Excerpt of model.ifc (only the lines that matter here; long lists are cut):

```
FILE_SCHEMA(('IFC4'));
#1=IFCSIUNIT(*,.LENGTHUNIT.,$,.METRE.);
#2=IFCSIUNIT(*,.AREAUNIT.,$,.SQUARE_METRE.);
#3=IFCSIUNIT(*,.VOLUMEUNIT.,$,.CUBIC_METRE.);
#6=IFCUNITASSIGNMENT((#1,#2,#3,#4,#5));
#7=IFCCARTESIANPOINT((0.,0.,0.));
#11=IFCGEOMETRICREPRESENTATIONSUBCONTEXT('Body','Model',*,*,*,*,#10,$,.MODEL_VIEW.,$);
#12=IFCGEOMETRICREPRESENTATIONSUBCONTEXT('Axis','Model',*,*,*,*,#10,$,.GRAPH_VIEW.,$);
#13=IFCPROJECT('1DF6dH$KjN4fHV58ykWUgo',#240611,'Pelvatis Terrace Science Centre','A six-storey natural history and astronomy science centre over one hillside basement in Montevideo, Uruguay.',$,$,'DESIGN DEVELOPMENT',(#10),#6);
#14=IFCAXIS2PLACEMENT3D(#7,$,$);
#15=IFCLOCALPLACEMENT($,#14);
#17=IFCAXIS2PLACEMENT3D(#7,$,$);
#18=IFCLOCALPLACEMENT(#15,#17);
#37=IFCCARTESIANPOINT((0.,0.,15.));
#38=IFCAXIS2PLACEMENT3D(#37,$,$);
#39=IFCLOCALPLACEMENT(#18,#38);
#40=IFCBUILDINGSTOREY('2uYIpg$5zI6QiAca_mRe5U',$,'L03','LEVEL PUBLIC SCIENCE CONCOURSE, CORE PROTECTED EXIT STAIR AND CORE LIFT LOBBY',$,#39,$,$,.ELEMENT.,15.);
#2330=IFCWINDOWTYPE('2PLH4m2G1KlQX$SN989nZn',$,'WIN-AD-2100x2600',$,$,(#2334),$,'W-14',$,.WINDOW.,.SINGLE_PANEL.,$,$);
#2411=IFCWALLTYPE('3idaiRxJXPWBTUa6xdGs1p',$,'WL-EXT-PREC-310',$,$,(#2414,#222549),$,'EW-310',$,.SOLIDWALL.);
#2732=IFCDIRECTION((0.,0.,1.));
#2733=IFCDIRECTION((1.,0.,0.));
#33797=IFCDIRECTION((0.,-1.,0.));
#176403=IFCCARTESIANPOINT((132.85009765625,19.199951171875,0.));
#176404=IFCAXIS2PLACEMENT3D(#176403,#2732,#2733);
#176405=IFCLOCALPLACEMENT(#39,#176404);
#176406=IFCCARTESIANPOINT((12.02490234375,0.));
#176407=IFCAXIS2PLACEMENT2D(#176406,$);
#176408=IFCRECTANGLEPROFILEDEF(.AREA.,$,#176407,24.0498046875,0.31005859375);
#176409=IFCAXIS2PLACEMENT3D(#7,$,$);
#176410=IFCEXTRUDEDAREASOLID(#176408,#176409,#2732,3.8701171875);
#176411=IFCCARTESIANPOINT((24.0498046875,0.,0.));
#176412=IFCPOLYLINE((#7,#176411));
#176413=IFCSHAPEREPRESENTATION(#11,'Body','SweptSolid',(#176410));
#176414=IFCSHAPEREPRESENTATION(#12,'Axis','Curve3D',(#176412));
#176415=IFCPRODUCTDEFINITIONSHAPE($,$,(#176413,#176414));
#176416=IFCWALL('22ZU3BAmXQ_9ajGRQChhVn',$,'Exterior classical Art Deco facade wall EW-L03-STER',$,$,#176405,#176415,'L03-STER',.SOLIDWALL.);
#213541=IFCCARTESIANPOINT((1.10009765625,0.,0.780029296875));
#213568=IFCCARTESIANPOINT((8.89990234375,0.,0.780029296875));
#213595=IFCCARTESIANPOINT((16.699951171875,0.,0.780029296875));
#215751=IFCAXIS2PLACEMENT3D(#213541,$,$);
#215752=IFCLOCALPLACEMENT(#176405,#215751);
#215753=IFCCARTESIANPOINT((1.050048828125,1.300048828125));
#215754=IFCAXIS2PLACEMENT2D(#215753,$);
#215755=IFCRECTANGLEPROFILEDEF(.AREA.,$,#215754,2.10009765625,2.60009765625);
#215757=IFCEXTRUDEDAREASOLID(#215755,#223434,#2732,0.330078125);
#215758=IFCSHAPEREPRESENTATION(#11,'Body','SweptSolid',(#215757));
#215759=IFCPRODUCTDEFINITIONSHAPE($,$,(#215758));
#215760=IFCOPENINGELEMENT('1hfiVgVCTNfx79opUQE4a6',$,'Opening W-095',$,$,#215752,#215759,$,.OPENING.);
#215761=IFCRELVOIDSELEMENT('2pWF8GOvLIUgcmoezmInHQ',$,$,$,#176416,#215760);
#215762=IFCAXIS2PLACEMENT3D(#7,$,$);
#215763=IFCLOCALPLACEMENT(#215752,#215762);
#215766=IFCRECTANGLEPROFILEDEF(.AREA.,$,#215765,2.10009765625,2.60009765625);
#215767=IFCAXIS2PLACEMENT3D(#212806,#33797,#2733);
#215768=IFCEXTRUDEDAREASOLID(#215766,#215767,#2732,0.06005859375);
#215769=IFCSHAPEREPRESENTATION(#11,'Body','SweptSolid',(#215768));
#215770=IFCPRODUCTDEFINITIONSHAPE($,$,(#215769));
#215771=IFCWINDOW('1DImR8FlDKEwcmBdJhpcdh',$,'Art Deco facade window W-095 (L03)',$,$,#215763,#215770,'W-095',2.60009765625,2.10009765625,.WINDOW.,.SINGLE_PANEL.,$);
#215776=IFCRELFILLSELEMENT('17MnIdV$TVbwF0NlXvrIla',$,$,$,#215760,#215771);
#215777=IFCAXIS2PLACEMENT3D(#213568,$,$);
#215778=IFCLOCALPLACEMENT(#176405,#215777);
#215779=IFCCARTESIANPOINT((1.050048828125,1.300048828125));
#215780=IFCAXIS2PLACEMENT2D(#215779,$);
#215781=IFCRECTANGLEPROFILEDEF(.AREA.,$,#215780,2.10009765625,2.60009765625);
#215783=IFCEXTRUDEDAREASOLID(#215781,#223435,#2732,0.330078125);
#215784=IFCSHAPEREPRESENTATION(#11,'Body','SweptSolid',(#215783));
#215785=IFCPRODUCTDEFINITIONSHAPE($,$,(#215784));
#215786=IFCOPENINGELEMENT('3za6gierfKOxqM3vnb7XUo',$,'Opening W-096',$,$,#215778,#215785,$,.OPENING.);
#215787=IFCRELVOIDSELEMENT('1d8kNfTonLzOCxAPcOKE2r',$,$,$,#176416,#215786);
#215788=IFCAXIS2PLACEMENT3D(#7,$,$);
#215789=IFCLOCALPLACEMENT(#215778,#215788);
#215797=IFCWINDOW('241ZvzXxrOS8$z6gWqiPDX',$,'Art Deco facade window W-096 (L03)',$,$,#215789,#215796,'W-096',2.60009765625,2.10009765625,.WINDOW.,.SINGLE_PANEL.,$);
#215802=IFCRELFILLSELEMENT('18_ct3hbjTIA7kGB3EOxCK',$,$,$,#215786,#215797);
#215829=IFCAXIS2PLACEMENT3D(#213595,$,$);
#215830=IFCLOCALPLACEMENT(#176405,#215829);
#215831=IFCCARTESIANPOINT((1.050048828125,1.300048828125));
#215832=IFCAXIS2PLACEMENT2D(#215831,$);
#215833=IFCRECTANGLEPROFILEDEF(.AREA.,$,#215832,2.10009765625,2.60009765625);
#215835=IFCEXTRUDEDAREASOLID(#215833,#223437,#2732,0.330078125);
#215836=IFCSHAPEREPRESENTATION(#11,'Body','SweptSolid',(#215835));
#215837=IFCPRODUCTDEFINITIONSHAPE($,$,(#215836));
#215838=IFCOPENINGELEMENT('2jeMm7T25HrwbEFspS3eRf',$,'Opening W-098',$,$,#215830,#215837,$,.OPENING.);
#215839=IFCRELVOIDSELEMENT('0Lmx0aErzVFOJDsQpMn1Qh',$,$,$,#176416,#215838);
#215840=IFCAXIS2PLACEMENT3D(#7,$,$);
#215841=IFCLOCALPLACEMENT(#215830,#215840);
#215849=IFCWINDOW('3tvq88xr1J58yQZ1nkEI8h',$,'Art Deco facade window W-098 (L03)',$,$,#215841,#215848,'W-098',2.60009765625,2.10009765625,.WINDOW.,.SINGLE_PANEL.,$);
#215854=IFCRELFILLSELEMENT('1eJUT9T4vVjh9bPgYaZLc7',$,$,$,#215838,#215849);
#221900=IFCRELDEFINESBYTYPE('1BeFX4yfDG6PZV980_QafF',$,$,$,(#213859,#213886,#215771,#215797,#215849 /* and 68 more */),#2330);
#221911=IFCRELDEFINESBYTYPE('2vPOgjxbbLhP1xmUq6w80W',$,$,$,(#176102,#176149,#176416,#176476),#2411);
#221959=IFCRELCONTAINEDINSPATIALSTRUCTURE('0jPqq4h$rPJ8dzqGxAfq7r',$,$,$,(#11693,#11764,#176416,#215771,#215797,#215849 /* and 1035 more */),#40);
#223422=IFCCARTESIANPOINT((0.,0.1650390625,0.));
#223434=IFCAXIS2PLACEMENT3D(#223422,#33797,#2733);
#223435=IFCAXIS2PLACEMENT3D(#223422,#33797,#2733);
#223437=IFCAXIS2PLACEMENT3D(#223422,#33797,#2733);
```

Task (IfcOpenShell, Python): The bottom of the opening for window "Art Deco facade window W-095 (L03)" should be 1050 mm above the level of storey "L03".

```python
import numpy as np
import ifcopenshell
import ifcopenshell.api.geometry
import ifcopenshell.geom
import ifcopenshell.util.element
import ifcopenshell.util.placement
import ifcopenshell.util.shape
import ifcopenshell.util.unit

model = ifcopenshell.open("model.ifc")
unit_scale = ifcopenshell.util.unit.calculate_unit_scale(model)

window = model.by_guid("1DImR8FlDKEwcmBdJhpcdh")
opening = window.FillsVoids[0].RelatingOpeningElement
storey = ifcopenshell.util.element.get_container(window, ifc_class="IfcBuildingStorey")
level = ifcopenshell.util.placement.get_local_placement(storey.ObjectPlacement)[2, 3]

# The opening's origin need not be at the sill, so measure its lowest point.
shape = ifcopenshell.geom.create_shape(ifcopenshell.geom.settings(), opening)
bottom = ifcopenshell.util.shape.get_shape_bottom_elevation(shape, shape.geometry) / unit_scale
dz = level + 1.05 - bottom

shift = np.array([0.0, 0.0, dz])
# The window is placed relative to its opening, so it follows when the opening moves.
matrix = ifcopenshell.util.placement.get_local_placement(opening.ObjectPlacement)
matrix[:3, 3] += shift
ifcopenshell.api.geometry.edit_object_placement(
    model, product=opening, matrix=matrix, is_si=False, should_transform_children=True
)

print(f"moved by {dz * unit_scale:+.3f} m")

model.write("model_edited.ifc")
```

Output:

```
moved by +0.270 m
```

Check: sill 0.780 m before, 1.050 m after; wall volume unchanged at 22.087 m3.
